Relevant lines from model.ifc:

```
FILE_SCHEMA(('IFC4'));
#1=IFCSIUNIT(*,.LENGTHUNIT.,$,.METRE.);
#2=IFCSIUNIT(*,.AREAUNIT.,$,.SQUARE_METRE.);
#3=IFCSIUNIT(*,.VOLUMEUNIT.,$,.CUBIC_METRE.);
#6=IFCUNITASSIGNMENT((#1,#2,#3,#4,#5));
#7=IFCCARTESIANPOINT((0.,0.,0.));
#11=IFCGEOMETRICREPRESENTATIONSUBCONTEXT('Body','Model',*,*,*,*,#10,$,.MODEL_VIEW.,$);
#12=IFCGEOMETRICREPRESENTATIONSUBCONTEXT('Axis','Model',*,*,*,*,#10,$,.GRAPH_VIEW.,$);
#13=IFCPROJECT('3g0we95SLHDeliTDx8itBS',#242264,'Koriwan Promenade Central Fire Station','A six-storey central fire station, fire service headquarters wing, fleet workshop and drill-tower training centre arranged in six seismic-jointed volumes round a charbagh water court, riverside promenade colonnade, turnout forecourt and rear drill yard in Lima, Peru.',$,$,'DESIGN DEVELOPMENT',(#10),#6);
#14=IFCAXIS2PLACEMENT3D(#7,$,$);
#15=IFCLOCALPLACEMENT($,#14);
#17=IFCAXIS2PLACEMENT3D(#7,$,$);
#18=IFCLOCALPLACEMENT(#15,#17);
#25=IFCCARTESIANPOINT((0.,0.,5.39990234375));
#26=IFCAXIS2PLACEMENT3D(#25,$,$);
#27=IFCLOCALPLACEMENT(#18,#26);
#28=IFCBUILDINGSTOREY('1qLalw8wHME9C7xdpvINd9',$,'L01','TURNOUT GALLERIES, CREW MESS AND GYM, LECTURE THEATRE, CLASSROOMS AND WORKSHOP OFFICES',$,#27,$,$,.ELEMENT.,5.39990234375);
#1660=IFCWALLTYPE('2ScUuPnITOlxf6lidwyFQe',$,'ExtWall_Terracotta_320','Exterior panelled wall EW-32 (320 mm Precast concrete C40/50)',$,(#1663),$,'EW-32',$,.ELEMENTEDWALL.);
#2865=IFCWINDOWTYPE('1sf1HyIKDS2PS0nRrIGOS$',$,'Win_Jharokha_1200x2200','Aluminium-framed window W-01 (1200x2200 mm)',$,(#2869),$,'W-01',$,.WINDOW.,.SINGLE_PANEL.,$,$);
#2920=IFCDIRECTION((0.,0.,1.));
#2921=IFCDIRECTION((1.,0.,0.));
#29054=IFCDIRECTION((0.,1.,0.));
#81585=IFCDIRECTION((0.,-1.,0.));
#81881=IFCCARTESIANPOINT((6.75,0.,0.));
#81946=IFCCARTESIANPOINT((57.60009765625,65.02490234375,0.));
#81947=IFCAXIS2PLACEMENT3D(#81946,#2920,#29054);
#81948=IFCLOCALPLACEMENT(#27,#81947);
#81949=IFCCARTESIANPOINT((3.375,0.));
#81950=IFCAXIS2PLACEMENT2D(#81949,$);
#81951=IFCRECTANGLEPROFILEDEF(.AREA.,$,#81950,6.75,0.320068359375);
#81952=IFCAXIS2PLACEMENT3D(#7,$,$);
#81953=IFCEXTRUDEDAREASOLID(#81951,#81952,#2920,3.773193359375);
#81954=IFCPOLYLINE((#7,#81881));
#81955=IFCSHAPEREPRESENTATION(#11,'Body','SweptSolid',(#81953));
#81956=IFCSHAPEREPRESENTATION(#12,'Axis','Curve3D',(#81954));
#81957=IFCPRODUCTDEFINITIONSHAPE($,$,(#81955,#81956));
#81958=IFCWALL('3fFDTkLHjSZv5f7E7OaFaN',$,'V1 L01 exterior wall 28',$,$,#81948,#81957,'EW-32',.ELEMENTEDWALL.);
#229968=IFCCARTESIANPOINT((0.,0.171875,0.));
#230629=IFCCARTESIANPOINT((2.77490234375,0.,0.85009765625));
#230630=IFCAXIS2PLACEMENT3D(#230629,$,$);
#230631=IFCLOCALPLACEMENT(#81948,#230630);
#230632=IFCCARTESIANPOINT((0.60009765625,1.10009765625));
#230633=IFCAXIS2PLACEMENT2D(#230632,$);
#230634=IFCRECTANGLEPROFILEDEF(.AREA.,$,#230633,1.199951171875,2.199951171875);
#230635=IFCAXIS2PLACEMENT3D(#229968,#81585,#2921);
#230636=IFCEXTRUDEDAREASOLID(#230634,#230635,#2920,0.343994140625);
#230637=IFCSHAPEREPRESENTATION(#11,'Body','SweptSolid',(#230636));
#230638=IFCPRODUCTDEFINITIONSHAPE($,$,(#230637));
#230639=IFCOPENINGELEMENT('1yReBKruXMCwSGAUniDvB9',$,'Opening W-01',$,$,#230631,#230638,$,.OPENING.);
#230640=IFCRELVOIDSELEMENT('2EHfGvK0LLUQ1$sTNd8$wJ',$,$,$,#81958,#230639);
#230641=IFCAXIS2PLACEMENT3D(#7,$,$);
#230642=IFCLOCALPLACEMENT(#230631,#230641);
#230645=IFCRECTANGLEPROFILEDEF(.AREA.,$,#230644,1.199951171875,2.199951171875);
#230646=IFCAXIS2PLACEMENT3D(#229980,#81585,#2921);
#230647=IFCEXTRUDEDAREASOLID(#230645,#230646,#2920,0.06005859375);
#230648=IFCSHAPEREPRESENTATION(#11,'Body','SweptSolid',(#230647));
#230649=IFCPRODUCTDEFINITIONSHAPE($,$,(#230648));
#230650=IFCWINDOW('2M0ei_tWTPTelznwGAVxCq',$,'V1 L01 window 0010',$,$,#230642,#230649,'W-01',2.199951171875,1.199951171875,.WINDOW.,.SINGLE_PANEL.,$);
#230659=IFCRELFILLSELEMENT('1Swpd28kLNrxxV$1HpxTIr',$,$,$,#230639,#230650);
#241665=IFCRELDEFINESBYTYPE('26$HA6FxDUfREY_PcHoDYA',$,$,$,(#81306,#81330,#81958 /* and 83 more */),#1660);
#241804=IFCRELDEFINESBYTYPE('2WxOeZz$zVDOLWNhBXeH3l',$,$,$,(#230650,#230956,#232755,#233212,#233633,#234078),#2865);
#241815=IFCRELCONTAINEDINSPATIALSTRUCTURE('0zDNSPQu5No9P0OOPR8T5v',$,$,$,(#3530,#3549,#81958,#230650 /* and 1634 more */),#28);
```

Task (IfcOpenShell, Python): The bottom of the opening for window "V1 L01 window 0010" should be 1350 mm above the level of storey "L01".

```python
import numpy as np
import ifcopenshell
import ifcopenshell.api.geometry
import ifcopenshell.geom
import ifcopenshell.util.element
import ifcopenshell.util.placement
import ifcopenshell.util.shape
import ifcopenshell.util.unit

model = ifcopenshell.open("model.ifc")
unit_scale = ifcopenshell.util.unit.calculate_unit_scale(model)

window = model.by_id(230650)
opening = window.FillsVoids[0].RelatingOpeningElement
storey = ifcopenshell.util.element.get_container(window, ifc_class="IfcBuildingStorey")
level = ifcopenshell.util.placement.get_local_placement(storey.ObjectPlacement)[2, 3]

# The opening's origin need not be at the sill, so measure its lowest point.
shape = ifcopenshell.geom.create_shape(ifcopenshell.geom.settings(), opening)
bottom = ifcopenshell.util.shape.get_shape_bottom_elevation(shape, shape.geometry) / unit_scale
dz = level + 1.35 / unit_scale - bottom

shift = np.array([0.0, 0.0, dz])
# The window is placed relative to its opening, so it follows when the opening moves.
matrix = ifcopenshell.util.placement.get_local_placement(opening.ObjectPlacement)
matrix[:3, 3] += shift
ifcopenshell.api.geometry.edit_object_placement(
    model, product=opening, matrix=matrix, is_si=False, should_transform_children=True
)

print(f"moved by {dz * unit_scale:+.3f} m")

model.write("model_updated.ifc")
```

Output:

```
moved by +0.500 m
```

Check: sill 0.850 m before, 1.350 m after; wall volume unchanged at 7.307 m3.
